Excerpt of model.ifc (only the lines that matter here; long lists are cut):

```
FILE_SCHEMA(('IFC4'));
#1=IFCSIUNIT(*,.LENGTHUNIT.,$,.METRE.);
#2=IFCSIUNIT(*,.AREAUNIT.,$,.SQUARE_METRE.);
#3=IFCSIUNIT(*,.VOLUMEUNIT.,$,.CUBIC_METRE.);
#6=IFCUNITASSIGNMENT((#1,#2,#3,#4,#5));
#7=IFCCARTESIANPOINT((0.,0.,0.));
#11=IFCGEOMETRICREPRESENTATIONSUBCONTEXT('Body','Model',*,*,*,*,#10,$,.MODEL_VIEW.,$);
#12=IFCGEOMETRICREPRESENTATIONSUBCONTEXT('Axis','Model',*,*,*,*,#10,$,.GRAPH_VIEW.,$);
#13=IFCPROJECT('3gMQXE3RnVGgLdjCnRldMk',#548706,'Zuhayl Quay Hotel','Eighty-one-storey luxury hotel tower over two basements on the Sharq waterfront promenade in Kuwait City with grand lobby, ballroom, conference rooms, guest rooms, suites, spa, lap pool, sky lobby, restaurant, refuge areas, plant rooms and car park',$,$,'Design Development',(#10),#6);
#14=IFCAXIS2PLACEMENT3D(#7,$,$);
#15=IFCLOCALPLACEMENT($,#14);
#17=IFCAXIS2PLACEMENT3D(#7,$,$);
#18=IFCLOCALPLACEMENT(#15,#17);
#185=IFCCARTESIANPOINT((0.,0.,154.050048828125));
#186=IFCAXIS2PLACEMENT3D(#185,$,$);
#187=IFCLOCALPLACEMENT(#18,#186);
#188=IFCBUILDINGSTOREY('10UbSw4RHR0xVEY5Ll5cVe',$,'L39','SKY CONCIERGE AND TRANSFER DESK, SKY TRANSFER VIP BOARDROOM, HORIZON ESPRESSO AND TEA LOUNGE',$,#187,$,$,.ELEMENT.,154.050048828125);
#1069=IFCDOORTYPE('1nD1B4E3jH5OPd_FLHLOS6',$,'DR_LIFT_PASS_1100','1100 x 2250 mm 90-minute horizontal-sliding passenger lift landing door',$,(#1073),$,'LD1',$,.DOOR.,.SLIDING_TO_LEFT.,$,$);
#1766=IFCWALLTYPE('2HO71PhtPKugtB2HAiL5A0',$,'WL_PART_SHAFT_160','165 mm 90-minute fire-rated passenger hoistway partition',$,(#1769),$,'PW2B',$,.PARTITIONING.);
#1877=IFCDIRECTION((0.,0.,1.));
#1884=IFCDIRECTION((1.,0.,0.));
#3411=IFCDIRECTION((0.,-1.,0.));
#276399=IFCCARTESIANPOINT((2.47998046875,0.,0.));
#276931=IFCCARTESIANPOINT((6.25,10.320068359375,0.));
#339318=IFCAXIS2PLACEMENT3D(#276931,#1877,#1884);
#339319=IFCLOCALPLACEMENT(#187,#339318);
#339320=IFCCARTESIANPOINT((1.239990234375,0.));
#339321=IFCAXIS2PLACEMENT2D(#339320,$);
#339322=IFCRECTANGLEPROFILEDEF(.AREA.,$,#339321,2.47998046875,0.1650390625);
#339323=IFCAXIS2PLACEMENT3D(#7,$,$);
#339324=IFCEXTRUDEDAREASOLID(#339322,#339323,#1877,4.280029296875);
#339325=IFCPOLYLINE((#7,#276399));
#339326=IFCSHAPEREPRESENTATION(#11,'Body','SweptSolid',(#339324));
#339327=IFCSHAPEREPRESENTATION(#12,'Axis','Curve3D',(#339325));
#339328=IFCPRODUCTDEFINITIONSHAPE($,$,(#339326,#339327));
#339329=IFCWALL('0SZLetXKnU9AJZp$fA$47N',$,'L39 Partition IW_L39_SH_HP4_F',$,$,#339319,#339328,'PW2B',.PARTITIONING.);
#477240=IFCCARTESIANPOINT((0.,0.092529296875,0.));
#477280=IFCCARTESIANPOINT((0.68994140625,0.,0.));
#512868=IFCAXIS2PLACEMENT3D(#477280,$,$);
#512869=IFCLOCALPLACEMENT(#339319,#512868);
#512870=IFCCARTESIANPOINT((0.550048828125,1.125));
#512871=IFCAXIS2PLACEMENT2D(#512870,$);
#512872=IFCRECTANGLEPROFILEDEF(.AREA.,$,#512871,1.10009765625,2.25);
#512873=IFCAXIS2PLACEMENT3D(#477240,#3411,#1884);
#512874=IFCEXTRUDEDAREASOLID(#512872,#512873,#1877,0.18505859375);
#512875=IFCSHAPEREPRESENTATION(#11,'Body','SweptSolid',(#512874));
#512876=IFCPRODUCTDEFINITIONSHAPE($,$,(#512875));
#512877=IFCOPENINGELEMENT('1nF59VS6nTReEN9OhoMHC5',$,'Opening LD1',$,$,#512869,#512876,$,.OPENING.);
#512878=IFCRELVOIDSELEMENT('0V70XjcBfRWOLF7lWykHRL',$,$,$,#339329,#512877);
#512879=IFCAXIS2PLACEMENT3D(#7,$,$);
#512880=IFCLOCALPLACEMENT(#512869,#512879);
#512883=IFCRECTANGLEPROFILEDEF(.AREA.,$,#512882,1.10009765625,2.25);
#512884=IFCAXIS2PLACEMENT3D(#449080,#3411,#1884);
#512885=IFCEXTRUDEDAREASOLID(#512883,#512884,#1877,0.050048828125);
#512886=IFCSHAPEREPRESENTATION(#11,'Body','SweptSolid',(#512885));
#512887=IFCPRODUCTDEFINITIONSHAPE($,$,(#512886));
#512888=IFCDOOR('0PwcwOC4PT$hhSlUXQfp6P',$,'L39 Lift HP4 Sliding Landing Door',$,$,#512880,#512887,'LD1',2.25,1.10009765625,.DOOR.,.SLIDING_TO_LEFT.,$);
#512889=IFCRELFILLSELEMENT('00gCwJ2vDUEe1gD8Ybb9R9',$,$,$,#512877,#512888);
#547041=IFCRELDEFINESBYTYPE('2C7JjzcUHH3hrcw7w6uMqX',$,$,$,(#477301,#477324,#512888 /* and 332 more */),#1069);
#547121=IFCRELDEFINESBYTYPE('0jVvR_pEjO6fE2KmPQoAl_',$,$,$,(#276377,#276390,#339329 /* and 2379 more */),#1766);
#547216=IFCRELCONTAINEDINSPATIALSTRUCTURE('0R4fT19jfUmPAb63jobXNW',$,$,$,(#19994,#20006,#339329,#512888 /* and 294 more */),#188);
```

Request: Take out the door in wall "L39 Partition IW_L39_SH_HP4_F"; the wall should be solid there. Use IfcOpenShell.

```python
import ifcopenshell
import ifcopenshell.api.feature
import ifcopenshell.api.root
import ifcopenshell.geom
import ifcopenshell.util.shape

model = ifcopenshell.open("model.ifc")
settings = ifcopenshell.geom.settings()


def volume(element):
    """Net volume in cubic metres, openings subtracted."""
    shape = ifcopenshell.geom.create_shape(settings, element)
    return ifcopenshell.util.shape.get_volume(shape.geometry)


door = model.by_guid("0PwcwOC4PT$hhSlUXQfp6P")
opening = door.FillsVoids[0].RelatingOpeningElement
wall = opening.VoidsElements[0].RelatingBuildingElement
before = volume(wall)

ifcopenshell.api.root.remove_product(model, product=door)
ifcopenshell.api.feature.remove_feature(model, feature=opening)

after = volume(wall)

print(f"wall volume {before:.3f} -> {after:.3f} m3")

model.write("model-out.ifc")
```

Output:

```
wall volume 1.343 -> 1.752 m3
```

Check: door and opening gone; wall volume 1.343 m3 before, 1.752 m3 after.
